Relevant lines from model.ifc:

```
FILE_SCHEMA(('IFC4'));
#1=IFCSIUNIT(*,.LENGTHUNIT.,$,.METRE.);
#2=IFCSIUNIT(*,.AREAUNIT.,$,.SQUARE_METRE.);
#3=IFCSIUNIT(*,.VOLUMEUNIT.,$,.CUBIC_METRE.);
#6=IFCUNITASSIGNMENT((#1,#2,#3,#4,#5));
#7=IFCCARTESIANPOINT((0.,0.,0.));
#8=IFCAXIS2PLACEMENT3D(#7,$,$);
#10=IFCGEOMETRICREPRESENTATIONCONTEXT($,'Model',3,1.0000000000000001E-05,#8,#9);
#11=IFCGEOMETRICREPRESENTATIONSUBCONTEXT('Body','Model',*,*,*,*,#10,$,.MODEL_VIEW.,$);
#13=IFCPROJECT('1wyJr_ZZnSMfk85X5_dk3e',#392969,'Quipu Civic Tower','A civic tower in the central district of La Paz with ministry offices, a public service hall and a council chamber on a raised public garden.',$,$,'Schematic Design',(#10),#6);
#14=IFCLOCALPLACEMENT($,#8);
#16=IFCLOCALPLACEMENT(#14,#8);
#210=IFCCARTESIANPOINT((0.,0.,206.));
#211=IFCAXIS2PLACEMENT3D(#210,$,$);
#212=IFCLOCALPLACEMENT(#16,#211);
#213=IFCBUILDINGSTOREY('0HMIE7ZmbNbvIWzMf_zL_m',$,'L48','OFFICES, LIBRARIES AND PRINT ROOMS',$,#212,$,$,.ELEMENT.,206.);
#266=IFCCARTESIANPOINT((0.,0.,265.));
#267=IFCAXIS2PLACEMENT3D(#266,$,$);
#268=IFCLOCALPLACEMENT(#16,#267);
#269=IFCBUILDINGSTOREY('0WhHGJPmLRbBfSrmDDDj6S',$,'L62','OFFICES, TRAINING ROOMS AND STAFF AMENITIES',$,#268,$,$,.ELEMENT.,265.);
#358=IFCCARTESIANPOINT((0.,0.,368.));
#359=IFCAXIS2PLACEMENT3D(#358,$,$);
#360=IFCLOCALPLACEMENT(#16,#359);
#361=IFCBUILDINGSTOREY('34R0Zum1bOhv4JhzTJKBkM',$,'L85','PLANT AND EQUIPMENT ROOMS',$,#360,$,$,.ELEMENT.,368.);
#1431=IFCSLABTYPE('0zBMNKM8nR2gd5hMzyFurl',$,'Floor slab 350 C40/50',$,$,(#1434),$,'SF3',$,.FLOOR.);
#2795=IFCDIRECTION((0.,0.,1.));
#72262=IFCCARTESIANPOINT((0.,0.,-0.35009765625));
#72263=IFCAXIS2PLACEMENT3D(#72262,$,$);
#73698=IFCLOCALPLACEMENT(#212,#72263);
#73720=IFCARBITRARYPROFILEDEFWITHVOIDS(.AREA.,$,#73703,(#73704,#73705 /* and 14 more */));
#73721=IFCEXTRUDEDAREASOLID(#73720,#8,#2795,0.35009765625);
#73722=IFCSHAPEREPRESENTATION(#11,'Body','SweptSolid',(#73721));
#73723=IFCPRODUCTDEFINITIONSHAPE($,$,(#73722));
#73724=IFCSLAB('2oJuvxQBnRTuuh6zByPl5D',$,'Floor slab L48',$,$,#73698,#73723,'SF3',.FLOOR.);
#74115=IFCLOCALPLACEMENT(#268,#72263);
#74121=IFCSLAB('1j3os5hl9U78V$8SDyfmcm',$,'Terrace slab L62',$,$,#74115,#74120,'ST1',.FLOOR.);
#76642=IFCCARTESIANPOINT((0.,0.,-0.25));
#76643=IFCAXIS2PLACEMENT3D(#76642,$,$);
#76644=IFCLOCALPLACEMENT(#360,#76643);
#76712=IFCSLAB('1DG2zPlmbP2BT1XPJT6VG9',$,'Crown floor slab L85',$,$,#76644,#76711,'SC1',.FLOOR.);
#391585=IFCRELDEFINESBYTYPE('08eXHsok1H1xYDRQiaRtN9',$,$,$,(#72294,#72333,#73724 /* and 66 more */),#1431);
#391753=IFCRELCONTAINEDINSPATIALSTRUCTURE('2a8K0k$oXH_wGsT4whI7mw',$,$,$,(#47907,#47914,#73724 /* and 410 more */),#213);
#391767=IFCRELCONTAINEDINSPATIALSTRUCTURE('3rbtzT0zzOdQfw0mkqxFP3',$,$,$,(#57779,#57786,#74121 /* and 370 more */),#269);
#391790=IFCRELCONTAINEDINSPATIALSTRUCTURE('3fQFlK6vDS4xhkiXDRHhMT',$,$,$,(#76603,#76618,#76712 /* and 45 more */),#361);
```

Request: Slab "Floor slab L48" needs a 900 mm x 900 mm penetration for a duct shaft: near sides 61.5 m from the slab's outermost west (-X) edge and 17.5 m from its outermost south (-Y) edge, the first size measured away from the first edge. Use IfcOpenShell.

```python
import numpy as np
import ifcopenshell
import ifcopenshell.api.feature
import ifcopenshell.api.geometry
import ifcopenshell.api.root
import ifcopenshell.geom
import ifcopenshell.util.placement
import ifcopenshell.util.representation
import ifcopenshell.util.shape
import ifcopenshell.util.unit

model = ifcopenshell.open("model.ifc")
unit_scale = ifcopenshell.util.unit.calculate_unit_scale(model)
settings = ifcopenshell.geom.settings()


def volume(element):
    """Net volume in cubic metres, openings subtracted."""
    shape = ifcopenshell.geom.create_shape(settings, element)
    return ifcopenshell.util.shape.get_volume(shape.geometry)


slab = model.by_guid("2oJuvxQBnRTuuh6zByPl5D")
before = volume(slab)

# Extent in the slab's own axes, in metres. The edges named are its -X and -Y sides.
slab_shape = ifcopenshell.geom.create_shape(settings, slab)
vertices = ifcopenshell.util.shape.get_vertices(slab_shape.geometry)
x_min, y_min, bottom = vertices.min(axis=0)
top = vertices[:, 2].max()

opening = ifcopenshell.api.root.create_entity(model, ifc_class="IfcOpeningElement", name="Duct shaft opening", predefined_type="OPENING")
context = ifcopenshell.util.representation.get_context(model, "Model", "Body", "MODEL_VIEW")
width, depth = 0.9, 0.9
outline = [(0.0, 0.0), (width, 0.0), (width, depth), (0.0, depth), (0.0, 0.0)]
# Overshoot both faces by 50 mm so the cut is clean.
shape = ifcopenshell.api.geometry.add_slab_representation(
    model, context=context, depth=top - bottom + 0.1, polyline=outline
)
ifcopenshell.api.geometry.assign_representation(model, product=opening, representation=shape)

matrix = ifcopenshell.util.placement.get_local_placement(slab.ObjectPlacement)
matrix[:, 3] = matrix @ np.append(np.array([x_min + 61.5, y_min + 17.5, bottom - 0.05]) / unit_scale, 1.0)
ifcopenshell.api.geometry.edit_object_placement(model, product=opening, matrix=matrix, is_si=False)
ifcopenshell.api.feature.add_feature(model, feature=opening, element=slab)

after = volume(slab)

print(f"slab volume {before:.3f} -> {after:.3f} m3")

model.write("model_v2.ifc")
```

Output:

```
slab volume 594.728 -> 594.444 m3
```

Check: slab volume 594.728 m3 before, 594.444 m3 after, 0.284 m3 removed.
